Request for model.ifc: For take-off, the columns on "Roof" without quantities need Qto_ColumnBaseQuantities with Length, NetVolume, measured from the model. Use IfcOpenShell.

First a look at what the model holds.

```python
import ifcopenshell
import ifcopenshell.util.element
import ifcopenshell.util.unit

model = ifcopenshell.open("model.ifc")
print(model.schema)
for unit_type in ("LENGTHUNIT", "AREAUNIT", "VOLUMEUNIT"):
    print(unit_type, ifcopenshell.util.unit.calculate_unit_scale(model, unit_type))
storey = next(s for s in model.by_type("IfcBuildingStorey") if s.Name == "Roof")
columns = [e for e in ifcopenshell.util.element.get_decomposition(storey) if e.is_a("IfcColumn")]
for e in sorted(columns, key=lambda e: e.id()):
    print(e.id(), e.is_a(), e.Name, list(ifcopenshell.util.element.get_psets(e, qtos_only=True)), sep=" | ")
```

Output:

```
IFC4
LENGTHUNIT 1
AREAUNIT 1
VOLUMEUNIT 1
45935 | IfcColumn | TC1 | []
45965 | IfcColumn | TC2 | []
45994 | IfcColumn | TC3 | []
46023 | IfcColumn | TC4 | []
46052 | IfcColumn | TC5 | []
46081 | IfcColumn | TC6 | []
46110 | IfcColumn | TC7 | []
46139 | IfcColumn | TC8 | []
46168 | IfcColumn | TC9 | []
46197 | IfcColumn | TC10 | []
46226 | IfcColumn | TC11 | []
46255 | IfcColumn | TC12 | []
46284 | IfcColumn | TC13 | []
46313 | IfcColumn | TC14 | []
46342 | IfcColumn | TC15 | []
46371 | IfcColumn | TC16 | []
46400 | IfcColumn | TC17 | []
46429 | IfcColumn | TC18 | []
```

```python
import ifcopenshell
import ifcopenshell.api.pset
import ifcopenshell.geom
import ifcopenshell.util.element
import ifcopenshell.util.shape
import ifcopenshell.util.unit

model = ifcopenshell.open("model.ifc")
unit_scale = ifcopenshell.util.unit.calculate_unit_scale(model)
volume_scale = ifcopenshell.util.unit.calculate_unit_scale(model, "VOLUMEUNIT")
settings = ifcopenshell.geom.settings()

storey = next(s for s in model.by_type("IfcBuildingStorey") if s.Name == "Roof")
columns = [e for e in ifcopenshell.util.element.get_decomposition(storey) if e.is_a("IfcColumn")]

for e in sorted(columns, key=lambda e: e.id()):
    if ifcopenshell.util.element.get_psets(e, qtos_only=True, should_inherit=False):
        continue
    # Geometry comes back in metres, in the element's own axes.
    shape = ifcopenshell.geom.create_shape(settings, e)
    values = {
        "Length": ifcopenshell.util.shape.get_z(shape.geometry) / unit_scale,
        "NetVolume": ifcopenshell.util.shape.get_volume(shape.geometry) / volume_scale,
    }
    qto = ifcopenshell.api.pset.add_qto(model, product=e, name="Qto_ColumnBaseQuantities")
    ifcopenshell.api.pset.edit_qto(model, qto=qto, properties=values)
    print(e.id(), {k: round(v, 3) for k, v in values.items()})

model.write("model_rev.ifc")
```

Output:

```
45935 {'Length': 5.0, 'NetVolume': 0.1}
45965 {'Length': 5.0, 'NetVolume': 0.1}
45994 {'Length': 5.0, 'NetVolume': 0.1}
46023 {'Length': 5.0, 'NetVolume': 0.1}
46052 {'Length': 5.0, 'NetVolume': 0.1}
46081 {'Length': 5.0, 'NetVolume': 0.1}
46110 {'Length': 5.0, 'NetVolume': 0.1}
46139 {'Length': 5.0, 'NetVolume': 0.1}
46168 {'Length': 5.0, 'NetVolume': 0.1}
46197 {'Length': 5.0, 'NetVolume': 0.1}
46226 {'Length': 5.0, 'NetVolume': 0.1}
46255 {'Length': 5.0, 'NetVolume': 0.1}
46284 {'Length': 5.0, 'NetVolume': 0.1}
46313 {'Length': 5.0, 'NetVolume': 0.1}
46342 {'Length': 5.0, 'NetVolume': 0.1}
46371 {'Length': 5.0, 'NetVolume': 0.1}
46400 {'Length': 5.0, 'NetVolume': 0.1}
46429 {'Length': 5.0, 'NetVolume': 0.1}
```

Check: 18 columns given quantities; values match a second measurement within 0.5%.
